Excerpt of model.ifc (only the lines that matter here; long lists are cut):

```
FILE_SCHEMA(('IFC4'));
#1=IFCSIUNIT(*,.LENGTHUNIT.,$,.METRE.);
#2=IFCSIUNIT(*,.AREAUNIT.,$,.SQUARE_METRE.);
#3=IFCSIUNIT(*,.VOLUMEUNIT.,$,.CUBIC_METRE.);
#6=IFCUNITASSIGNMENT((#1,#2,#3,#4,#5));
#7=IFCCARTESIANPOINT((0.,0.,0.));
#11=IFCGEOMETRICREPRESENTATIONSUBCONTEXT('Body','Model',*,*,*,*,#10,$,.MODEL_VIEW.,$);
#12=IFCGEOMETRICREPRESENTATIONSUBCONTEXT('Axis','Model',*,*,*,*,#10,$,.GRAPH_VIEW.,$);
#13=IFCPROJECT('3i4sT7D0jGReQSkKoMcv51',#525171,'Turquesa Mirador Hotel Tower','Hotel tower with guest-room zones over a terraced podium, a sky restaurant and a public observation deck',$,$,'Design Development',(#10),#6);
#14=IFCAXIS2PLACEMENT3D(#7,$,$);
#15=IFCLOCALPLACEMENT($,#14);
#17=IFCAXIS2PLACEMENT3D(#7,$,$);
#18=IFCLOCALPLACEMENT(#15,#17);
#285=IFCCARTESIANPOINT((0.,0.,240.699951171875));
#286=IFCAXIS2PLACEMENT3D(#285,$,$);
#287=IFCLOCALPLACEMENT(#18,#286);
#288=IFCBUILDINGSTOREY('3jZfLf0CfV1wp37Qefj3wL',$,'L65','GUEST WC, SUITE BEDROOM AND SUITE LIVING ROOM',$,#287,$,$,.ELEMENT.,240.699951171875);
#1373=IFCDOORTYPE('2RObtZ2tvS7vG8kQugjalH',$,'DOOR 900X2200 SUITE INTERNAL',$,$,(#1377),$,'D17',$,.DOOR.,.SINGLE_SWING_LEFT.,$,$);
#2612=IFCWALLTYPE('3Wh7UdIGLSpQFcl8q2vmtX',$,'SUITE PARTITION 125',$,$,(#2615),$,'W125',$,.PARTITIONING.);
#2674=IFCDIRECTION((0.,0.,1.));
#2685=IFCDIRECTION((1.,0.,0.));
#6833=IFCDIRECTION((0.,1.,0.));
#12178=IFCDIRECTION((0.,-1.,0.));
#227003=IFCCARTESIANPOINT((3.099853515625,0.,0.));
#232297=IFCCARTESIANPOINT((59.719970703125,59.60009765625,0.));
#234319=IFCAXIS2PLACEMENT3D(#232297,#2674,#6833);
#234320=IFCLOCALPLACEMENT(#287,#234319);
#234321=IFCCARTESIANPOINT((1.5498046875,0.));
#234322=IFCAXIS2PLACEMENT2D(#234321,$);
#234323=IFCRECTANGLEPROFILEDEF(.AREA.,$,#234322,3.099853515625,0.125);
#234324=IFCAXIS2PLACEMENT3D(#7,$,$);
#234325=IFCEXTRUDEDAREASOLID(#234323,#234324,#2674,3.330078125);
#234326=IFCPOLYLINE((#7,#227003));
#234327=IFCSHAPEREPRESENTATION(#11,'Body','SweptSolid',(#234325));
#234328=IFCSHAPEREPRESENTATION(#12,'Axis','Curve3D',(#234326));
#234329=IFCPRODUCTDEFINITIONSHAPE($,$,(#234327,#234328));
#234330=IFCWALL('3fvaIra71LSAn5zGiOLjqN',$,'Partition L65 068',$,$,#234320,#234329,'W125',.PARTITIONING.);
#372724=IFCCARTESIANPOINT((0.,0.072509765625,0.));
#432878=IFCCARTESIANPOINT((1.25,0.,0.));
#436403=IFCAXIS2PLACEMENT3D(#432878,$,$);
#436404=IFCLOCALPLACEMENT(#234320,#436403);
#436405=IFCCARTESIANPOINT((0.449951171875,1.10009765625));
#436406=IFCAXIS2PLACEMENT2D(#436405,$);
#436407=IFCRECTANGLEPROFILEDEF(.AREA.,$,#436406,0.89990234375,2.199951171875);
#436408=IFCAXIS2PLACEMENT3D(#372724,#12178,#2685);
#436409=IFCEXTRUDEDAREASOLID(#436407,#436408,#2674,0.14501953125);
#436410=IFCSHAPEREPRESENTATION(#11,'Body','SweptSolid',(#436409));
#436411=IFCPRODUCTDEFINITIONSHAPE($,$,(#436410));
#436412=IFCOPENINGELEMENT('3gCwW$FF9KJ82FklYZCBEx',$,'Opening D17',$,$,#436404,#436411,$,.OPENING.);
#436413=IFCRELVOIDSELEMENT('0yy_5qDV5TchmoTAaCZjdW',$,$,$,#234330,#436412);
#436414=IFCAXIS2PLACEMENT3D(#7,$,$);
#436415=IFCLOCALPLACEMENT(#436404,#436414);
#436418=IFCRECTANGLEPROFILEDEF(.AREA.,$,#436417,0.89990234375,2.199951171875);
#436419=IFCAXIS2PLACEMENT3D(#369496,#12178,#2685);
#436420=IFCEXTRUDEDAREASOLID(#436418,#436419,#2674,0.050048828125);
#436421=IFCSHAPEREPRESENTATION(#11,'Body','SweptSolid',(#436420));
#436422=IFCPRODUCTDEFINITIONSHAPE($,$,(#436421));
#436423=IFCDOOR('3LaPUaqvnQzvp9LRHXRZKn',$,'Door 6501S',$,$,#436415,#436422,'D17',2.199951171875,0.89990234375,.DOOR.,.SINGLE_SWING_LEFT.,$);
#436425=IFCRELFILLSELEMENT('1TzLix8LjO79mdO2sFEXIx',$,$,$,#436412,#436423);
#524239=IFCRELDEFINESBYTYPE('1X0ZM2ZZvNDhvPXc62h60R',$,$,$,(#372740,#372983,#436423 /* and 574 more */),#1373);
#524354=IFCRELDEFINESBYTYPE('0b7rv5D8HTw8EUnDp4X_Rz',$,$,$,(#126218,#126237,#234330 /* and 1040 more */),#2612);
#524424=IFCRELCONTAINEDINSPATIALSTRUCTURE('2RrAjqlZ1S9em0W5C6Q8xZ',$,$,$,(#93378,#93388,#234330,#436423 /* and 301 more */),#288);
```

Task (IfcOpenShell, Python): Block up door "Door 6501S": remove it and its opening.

```python
import ifcopenshell
import ifcopenshell.api.feature
import ifcopenshell.api.root
import ifcopenshell.geom
import ifcopenshell.util.shape

model = ifcopenshell.open("model.ifc")
settings = ifcopenshell.geom.settings()


def volume(element):
    """Net volume in cubic metres, openings subtracted."""
    shape = ifcopenshell.geom.create_shape(settings, element)
    return ifcopenshell.util.shape.get_volume(shape.geometry)


door = model.by_id(436423)
opening = door.FillsVoids[0].RelatingOpeningElement
wall = opening.VoidsElements[0].RelatingBuildingElement
before = volume(wall)

ifcopenshell.api.root.remove_product(model, product=door)
ifcopenshell.api.feature.remove_feature(model, feature=opening)

after = volume(wall)

print(f"wall volume {before:.3f} -> {after:.3f} m3")

model.write("model_updated.ifc")
```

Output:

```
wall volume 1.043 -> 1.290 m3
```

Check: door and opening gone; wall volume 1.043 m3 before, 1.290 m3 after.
